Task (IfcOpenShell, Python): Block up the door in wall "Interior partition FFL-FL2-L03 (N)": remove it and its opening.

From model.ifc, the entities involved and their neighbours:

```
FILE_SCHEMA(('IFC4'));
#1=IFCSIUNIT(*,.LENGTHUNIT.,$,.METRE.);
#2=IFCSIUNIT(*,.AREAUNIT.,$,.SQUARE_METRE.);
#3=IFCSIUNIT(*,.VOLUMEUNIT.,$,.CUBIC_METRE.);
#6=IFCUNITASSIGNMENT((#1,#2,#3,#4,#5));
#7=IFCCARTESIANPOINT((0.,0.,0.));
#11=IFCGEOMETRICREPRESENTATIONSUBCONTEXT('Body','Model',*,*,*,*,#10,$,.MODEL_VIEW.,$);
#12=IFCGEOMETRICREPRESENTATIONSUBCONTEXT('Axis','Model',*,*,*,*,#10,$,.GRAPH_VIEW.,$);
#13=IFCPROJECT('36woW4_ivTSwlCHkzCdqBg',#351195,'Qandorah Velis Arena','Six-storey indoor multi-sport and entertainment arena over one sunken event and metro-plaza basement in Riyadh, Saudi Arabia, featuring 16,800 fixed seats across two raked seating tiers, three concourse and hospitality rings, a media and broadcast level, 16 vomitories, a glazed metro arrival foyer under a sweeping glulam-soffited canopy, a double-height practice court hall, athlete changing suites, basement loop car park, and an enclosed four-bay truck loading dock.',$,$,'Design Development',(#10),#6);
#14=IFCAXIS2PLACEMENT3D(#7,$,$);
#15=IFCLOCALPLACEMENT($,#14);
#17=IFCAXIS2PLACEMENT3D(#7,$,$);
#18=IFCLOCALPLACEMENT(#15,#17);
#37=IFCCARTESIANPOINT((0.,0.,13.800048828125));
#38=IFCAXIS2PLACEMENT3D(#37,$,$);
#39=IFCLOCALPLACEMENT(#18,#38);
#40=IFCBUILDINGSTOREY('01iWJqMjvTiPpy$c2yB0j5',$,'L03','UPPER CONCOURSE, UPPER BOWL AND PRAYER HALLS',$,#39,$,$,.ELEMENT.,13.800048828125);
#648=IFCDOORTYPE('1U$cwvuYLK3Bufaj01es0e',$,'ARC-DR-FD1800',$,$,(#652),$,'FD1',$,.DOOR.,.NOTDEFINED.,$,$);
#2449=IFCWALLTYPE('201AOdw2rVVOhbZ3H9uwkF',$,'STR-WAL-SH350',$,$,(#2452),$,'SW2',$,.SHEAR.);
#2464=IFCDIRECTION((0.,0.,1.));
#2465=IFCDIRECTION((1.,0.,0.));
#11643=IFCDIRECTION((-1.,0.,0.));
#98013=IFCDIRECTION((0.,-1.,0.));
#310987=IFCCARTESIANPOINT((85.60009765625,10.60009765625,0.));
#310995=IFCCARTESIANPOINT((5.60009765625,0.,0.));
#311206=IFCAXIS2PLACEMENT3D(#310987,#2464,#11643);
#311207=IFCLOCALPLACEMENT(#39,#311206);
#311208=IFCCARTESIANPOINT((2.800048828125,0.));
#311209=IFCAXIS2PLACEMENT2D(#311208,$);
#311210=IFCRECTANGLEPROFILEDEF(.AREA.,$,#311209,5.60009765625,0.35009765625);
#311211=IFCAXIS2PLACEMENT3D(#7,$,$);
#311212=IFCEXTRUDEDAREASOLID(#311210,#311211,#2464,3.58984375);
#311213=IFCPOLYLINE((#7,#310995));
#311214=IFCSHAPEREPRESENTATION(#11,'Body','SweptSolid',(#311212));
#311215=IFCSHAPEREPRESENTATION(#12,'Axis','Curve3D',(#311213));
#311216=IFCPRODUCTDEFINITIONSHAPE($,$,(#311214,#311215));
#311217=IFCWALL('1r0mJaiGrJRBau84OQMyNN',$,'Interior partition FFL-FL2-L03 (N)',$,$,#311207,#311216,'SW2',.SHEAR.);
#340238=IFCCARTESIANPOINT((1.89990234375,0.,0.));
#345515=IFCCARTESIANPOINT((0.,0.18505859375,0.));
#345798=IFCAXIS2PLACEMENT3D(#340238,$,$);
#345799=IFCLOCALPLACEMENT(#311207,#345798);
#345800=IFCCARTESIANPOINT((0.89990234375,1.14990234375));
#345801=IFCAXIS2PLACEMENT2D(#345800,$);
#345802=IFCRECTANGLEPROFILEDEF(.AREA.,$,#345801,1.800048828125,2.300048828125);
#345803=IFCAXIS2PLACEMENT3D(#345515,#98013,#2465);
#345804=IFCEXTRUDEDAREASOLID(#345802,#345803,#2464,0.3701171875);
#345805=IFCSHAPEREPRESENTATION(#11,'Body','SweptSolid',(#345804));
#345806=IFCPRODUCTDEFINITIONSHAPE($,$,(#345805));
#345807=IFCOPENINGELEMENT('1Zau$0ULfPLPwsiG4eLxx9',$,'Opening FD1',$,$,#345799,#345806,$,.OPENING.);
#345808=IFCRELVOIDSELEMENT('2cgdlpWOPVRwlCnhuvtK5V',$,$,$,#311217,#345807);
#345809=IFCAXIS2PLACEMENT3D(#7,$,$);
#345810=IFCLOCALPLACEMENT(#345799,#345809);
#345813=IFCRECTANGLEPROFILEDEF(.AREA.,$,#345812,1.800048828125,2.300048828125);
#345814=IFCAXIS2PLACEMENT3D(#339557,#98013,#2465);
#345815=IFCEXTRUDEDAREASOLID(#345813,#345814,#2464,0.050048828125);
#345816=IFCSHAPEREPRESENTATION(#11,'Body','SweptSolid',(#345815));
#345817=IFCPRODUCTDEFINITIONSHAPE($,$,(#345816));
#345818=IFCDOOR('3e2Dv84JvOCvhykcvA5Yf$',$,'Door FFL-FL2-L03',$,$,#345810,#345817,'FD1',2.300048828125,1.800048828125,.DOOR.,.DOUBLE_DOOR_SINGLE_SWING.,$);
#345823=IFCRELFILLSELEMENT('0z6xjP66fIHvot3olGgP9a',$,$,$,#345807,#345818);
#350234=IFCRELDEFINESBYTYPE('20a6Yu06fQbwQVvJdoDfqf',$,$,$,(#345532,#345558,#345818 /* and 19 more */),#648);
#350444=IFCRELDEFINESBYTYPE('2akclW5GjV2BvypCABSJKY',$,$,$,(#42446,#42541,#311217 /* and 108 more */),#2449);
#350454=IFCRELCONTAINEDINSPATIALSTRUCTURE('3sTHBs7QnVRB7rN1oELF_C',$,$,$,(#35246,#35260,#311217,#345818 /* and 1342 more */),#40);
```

```python
import ifcopenshell
import ifcopenshell.api.feature
import ifcopenshell.api.root
import ifcopenshell.geom
import ifcopenshell.util.shape

model = ifcopenshell.open("model.ifc")
settings = ifcopenshell.geom.settings()


def volume(element):
    """Net volume in cubic metres, openings subtracted."""
    shape = ifcopenshell.geom.create_shape(settings, element)
    return ifcopenshell.util.shape.get_volume(shape.geometry)


door = model.by_id(345818)
opening = door.FillsVoids[0].RelatingOpeningElement
wall = opening.VoidsElements[0].RelatingBuildingElement
before = volume(wall)

ifcopenshell.api.root.remove_product(model, product=door)
ifcopenshell.api.feature.remove_feature(model, feature=opening)

after = volume(wall)

print(f"wall volume {before:.3f} -> {after:.3f} m3")

model.write("model_updated.ifc")
```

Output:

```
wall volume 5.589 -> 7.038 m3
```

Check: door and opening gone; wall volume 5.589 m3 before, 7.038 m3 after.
